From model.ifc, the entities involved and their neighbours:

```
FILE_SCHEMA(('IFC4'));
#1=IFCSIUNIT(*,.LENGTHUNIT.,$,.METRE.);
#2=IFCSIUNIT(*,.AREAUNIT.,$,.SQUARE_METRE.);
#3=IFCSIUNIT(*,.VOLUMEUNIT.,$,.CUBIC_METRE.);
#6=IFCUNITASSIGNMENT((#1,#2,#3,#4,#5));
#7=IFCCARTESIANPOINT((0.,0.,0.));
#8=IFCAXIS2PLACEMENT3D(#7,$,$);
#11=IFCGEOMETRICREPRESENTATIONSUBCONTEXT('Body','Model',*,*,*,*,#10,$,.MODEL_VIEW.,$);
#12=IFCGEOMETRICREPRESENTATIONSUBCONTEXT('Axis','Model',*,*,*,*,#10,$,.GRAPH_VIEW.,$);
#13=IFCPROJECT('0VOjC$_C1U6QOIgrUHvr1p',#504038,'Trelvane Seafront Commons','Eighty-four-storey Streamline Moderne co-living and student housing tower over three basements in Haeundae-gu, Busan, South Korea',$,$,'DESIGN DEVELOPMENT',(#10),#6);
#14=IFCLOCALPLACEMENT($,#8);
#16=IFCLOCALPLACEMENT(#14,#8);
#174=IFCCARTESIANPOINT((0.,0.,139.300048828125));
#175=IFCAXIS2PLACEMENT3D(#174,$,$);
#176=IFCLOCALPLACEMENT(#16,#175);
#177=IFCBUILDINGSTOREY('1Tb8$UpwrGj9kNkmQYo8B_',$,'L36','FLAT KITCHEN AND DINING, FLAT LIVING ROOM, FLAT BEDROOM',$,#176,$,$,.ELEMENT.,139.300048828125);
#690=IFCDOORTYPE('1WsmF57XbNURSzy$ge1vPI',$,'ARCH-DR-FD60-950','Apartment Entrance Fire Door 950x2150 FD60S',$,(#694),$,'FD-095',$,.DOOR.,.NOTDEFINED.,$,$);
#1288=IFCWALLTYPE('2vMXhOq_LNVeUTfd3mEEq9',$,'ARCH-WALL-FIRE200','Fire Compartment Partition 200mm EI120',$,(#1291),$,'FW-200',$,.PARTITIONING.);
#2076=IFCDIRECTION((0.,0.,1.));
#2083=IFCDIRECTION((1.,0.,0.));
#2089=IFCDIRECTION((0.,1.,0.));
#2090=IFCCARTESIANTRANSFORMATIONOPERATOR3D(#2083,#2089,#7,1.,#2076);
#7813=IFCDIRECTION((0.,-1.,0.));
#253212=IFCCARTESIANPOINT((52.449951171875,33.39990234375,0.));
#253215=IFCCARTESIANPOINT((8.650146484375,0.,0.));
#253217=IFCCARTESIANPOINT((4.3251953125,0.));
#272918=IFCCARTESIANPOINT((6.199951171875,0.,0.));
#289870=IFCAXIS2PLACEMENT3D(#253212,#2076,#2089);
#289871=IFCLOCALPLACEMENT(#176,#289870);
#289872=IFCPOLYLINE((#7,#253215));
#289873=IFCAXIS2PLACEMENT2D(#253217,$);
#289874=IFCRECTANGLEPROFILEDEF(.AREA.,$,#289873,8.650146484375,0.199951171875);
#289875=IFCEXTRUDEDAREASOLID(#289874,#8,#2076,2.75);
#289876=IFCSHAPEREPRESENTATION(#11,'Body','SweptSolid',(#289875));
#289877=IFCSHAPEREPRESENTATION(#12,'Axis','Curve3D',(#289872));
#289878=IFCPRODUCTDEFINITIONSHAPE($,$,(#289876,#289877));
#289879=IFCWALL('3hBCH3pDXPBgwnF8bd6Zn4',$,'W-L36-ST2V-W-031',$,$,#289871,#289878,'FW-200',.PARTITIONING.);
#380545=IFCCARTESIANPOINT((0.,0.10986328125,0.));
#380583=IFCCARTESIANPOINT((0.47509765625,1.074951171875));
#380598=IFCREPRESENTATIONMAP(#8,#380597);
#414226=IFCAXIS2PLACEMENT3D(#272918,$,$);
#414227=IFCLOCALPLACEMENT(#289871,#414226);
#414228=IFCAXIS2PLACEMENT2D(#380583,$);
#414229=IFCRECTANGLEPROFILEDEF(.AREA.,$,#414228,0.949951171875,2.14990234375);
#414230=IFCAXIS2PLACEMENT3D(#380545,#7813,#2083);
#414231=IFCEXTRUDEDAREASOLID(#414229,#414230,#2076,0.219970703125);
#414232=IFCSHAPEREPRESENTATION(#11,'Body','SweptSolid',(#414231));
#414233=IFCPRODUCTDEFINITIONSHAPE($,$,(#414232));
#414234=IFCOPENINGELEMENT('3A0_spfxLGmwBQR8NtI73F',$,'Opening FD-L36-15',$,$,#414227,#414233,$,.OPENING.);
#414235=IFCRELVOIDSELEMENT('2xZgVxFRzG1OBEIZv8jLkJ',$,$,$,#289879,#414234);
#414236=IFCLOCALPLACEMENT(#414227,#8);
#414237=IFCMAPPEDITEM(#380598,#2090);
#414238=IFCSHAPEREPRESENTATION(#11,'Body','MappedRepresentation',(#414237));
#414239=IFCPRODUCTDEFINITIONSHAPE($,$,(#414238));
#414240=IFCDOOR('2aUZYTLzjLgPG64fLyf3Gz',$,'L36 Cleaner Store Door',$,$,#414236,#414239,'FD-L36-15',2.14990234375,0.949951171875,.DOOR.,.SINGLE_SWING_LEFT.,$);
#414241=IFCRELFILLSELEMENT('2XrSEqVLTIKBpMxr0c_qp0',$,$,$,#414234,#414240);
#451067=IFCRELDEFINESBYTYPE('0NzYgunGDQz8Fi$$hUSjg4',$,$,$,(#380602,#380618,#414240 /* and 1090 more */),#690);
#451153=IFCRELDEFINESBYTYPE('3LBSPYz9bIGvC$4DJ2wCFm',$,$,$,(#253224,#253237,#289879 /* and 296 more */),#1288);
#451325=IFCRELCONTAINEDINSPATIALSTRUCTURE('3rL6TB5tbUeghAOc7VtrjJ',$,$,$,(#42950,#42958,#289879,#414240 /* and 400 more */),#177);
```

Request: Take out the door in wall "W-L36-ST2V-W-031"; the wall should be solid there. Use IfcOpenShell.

```python
import ifcopenshell
import ifcopenshell.api.feature
import ifcopenshell.api.root
import ifcopenshell.geom
import ifcopenshell.util.shape

model = ifcopenshell.open("model.ifc")
settings = ifcopenshell.geom.settings()


def volume(element):
    """Net volume in cubic metres, openings subtracted."""
    shape = ifcopenshell.geom.create_shape(settings, element)
    return ifcopenshell.util.shape.get_volume(shape.geometry)


door = model.by_id(414240)
opening = door.FillsVoids[0].RelatingOpeningElement
wall = opening.VoidsElements[0].RelatingBuildingElement
before = volume(wall)

ifcopenshell.api.root.remove_product(model, product=door)
ifcopenshell.api.feature.remove_feature(model, feature=opening)

after = volume(wall)

print(f"wall volume {before:.3f} -> {after:.3f} m3")

model.write("model-out.ifc")
```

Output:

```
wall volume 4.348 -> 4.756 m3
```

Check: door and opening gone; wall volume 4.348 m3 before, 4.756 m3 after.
